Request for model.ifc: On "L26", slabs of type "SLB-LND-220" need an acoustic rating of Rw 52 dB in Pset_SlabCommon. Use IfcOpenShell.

First a look at what the model holds.

```python
import ifcopenshell
import ifcopenshell.util.element

model = ifcopenshell.open("model.ifc")
print(model.schema)
storey = next(s for s in model.by_type("IfcBuildingStorey") if s.Name == "L26")
slabs = [e for e in ifcopenshell.util.element.get_decomposition(storey) if e.is_a("IfcSlab")]
seen = {}
for e in slabs:
    element_type = ifcopenshell.util.element.get_type(e)
    key = (element_type.Name if element_type != e and element_type else None, ifcopenshell.util.element.get_pset(e, "Pset_SlabCommon", "AcousticRating"))
    seen[key] = seen.get(key, 0) + 1
for (name, value), count in sorted(seen.items(), key=str):
    print(count, "x", name, "|", value)
```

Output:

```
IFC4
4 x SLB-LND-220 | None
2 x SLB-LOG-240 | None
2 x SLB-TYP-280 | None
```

```python
import ifcopenshell
import ifcopenshell.api.pset
import ifcopenshell.util.element

model = ifcopenshell.open("model.ifc")

storey = next(s for s in model.by_type("IfcBuildingStorey") if s.Name == "L26")
slabs = [e for e in ifcopenshell.util.element.get_decomposition(storey) if e.is_a("IfcSlab")]

count = 0
for e in slabs:
    element_type = ifcopenshell.util.element.get_type(e)
    if element_type in (None, e) or element_type.Name != "SLB-LND-220":
        continue
    found = ifcopenshell.util.element.get_pset(e, "Pset_SlabCommon", should_inherit=False)
    if found:
        pset = model.by_id(found["id"])
        if len(ifcopenshell.util.element.get_elements_by_pset(pset)) > 1:
            pset = ifcopenshell.api.pset.unshare_pset(model, products=[e], pset=pset)[0]
    else:
        pset = ifcopenshell.api.pset.add_pset(model, product=e, name="Pset_SlabCommon")
    ifcopenshell.api.pset.edit_pset(model, pset=pset, properties={"AcousticRating": "Rw 52 dB"})
    count += 1

print(count, "slabs updated")

model.write("model_rev.ifc")
```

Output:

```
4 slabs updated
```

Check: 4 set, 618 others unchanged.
